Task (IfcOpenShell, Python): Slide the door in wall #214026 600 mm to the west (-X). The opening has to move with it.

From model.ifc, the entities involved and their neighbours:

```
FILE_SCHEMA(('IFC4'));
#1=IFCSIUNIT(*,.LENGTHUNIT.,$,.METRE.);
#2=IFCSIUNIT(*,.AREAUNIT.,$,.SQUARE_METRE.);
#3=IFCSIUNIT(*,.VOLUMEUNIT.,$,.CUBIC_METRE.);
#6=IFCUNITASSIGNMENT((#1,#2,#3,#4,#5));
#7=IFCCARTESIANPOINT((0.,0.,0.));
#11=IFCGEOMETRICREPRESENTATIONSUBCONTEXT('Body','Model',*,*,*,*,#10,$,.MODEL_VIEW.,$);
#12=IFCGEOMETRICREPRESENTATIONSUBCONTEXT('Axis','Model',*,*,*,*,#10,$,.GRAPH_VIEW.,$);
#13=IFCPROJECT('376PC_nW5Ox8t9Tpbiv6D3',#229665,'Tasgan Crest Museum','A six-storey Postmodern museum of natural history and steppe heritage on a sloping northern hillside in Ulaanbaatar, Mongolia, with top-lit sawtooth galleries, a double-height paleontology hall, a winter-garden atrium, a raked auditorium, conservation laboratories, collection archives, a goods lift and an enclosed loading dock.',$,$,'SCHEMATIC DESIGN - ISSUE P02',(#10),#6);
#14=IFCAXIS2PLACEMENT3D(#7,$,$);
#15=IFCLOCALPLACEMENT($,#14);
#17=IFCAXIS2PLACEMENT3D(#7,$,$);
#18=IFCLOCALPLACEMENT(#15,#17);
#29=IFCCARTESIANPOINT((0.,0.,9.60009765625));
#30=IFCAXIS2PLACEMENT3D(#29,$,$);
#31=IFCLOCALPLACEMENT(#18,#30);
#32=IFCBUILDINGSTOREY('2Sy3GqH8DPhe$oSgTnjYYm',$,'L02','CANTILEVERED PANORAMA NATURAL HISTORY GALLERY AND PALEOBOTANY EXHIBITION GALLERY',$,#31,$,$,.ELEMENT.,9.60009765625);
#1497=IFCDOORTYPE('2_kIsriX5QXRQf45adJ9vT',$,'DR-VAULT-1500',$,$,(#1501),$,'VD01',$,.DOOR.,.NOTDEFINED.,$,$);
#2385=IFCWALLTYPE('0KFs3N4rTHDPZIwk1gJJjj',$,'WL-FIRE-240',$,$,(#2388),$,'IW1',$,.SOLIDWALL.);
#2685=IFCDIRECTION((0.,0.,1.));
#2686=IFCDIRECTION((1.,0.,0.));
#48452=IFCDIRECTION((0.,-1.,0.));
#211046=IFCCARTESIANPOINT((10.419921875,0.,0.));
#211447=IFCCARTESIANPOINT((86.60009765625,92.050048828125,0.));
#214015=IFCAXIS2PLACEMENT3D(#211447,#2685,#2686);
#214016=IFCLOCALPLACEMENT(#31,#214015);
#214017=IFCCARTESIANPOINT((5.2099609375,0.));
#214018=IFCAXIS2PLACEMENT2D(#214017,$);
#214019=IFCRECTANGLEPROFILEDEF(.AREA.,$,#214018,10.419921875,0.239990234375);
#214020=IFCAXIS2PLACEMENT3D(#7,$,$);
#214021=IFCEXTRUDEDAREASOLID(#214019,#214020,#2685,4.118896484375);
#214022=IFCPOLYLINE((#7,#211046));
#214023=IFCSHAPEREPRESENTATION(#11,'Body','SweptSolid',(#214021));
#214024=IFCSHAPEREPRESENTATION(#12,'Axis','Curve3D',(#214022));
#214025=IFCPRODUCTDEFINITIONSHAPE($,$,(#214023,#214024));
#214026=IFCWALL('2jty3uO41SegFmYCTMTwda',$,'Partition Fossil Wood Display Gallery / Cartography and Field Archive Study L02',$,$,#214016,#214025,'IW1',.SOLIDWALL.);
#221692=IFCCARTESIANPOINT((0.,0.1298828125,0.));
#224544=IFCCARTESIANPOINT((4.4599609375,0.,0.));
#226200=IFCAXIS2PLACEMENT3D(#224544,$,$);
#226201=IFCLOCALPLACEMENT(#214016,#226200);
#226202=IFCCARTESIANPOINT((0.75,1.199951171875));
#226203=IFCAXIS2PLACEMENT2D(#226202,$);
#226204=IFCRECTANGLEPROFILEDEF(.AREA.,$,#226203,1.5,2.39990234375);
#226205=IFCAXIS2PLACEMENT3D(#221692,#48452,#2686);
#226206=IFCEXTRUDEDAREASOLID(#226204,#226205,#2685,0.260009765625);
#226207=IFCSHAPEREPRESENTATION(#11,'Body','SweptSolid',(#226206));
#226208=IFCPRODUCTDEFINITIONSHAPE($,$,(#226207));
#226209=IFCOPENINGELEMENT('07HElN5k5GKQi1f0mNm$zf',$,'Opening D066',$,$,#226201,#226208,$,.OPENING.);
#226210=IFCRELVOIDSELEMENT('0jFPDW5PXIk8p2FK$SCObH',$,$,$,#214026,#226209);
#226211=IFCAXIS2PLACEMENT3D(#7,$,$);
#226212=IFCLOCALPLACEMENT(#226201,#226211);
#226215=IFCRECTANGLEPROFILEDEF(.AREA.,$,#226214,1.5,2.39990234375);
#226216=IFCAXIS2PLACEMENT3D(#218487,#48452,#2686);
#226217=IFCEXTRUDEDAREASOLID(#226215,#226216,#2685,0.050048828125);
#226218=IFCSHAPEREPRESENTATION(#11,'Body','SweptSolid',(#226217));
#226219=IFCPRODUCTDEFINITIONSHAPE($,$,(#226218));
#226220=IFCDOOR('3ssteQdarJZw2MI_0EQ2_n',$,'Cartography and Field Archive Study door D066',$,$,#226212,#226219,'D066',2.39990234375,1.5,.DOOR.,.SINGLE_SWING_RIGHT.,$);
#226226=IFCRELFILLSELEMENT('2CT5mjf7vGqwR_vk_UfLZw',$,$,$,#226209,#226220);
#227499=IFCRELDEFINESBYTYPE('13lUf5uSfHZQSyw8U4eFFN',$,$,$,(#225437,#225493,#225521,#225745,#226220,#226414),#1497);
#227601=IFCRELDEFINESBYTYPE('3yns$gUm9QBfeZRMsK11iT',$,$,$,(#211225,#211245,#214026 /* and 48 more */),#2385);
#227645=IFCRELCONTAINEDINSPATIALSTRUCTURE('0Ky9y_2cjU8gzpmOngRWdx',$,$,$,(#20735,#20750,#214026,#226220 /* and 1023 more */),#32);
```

```python
import ifcopenshell
import ifcopenshell.api.geometry
import ifcopenshell.util.placement
import ifcopenshell.util.unit

model = ifcopenshell.open("model.ifc")
unit_scale = ifcopenshell.util.unit.calculate_unit_scale(model)

door = model.by_guid("3ssteQdarJZw2MI_0EQ2_n")
opening = door.FillsVoids[0].RelatingOpeningElement
wall = opening.VoidsElements[0].RelatingBuildingElement

wall_matrix = ifcopenshell.util.placement.get_local_placement(wall.ObjectPlacement)
shift = wall_matrix[:3, 0] * -0.6 / unit_scale
before = ifcopenshell.util.placement.get_local_placement(door.ObjectPlacement)[:3, 3].copy()

# The door is placed relative to its opening, so it follows when the opening moves.
matrix = ifcopenshell.util.placement.get_local_placement(opening.ObjectPlacement)
matrix[:3, 3] += shift
ifcopenshell.api.geometry.edit_object_placement(
    model, product=opening, matrix=matrix, is_si=False, should_transform_children=True
)

after = ifcopenshell.util.placement.get_local_placement(door.ObjectPlacement)[:3, 3]
print("door moved by", (after - before).round(3) + 0.0)

model.write("model_updated.ifc")
```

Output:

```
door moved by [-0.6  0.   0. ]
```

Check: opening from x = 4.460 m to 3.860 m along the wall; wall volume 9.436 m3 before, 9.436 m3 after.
